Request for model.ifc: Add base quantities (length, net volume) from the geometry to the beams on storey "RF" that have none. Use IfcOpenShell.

First a look at what the model holds.

```python
import ifcopenshell
import ifcopenshell.util.element
import ifcopenshell.util.unit

model = ifcopenshell.open("model.ifc")
print(model.schema)
for unit_type in ("LENGTHUNIT", "AREAUNIT", "VOLUMEUNIT"):
    print(unit_type, ifcopenshell.util.unit.calculate_unit_scale(model, unit_type))
storey = next(s for s in model.by_type("IfcBuildingStorey") if s.Name == "RF")
beams = [e for e in ifcopenshell.util.element.get_decomposition(storey) if e.is_a("IfcBeam")]
for e in sorted(beams, key=lambda e: e.id()):
    print(e.id(), e.is_a(), e.Name, list(ifcopenshell.util.element.get_psets(e, qtos_only=True)), sep=" | ")
```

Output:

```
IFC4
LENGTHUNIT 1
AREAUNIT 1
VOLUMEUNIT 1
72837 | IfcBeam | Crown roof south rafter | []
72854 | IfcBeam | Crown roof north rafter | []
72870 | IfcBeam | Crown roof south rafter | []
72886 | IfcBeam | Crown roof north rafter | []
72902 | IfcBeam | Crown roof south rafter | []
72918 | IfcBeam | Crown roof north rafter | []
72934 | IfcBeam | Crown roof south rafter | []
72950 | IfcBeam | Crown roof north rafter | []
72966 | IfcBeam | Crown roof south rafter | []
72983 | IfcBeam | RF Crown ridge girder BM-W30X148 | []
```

```python
import ifcopenshell
import ifcopenshell.api.pset
import ifcopenshell.geom
import ifcopenshell.util.element
import ifcopenshell.util.shape
import ifcopenshell.util.unit

model = ifcopenshell.open("model.ifc")
unit_scale = ifcopenshell.util.unit.calculate_unit_scale(model)
volume_scale = ifcopenshell.util.unit.calculate_unit_scale(model, "VOLUMEUNIT")
settings = ifcopenshell.geom.settings()

storey = next(s for s in model.by_type("IfcBuildingStorey") if s.Name == "RF")
beams = [e for e in ifcopenshell.util.element.get_decomposition(storey) if e.is_a("IfcBeam")]

for e in sorted(beams, key=lambda e: e.id()):
    if ifcopenshell.util.element.get_psets(e, qtos_only=True, should_inherit=False):
        continue
    # Geometry comes back in metres, in the element's own axes.
    shape = ifcopenshell.geom.create_shape(settings, e)
    values = {
        "Length": ifcopenshell.util.shape.get_max_xyz(shape.geometry) / unit_scale,
        "NetVolume": ifcopenshell.util.shape.get_volume(shape.geometry) / volume_scale,
    }
    qto = ifcopenshell.api.pset.add_qto(model, product=e, name="Qto_BeamBaseQuantities")
    ifcopenshell.api.pset.edit_qto(model, qto=qto, properties=values)
    print(e.id(), {k: round(v, 3) for k, v in values.items()})

model.write("model_rev.ifc")
```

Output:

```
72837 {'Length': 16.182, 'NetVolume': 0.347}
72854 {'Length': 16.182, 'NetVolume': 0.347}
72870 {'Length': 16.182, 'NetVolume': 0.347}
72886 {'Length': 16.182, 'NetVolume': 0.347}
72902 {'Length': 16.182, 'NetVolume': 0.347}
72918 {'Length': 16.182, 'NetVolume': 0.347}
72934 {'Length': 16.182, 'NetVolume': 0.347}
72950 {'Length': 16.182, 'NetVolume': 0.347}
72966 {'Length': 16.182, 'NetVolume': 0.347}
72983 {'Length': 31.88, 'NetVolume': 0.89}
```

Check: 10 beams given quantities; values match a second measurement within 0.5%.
